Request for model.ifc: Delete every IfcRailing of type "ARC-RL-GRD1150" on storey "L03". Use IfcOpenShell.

First a look at what the model holds.

```python
import ifcopenshell
import ifcopenshell.util.element

model = ifcopenshell.open("model.ifc")
print(model.schema)
storey = next(s for s in model.by_type("IfcBuildingStorey") if s.Name == "L03")
railings = [e for e in ifcopenshell.util.element.get_decomposition(storey) if e.is_a("IfcRailing")]
seen = {}
for e in railings:
    element_type = ifcopenshell.util.element.get_type(e)
    name = element_type.Name if element_type not in (None, e) else None
    seen[name] = seen.get(name, 0) + 1
for name, count in sorted(seen.items(), key=str):
    print(count, "x", name)
```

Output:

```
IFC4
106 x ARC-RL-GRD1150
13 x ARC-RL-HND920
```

```python
import ifcopenshell
import ifcopenshell.api.root
import ifcopenshell.util.element

model = ifcopenshell.open("model.ifc")

storey = next(s for s in model.by_type("IfcBuildingStorey") if s.Name == "L03")
railings = [e for e in ifcopenshell.util.element.get_decomposition(storey) if e.is_a("IfcRailing")]
targets = [e for e in railings if (t := ifcopenshell.util.element.get_type(e)) not in (None, e) and t.Name == "ARC-RL-GRD1150"]

for e in targets:
    ifcopenshell.api.root.remove_product(model, product=e)
print(len(targets), "removed")

model.write("model_edited.ifc")
```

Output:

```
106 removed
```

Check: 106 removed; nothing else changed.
